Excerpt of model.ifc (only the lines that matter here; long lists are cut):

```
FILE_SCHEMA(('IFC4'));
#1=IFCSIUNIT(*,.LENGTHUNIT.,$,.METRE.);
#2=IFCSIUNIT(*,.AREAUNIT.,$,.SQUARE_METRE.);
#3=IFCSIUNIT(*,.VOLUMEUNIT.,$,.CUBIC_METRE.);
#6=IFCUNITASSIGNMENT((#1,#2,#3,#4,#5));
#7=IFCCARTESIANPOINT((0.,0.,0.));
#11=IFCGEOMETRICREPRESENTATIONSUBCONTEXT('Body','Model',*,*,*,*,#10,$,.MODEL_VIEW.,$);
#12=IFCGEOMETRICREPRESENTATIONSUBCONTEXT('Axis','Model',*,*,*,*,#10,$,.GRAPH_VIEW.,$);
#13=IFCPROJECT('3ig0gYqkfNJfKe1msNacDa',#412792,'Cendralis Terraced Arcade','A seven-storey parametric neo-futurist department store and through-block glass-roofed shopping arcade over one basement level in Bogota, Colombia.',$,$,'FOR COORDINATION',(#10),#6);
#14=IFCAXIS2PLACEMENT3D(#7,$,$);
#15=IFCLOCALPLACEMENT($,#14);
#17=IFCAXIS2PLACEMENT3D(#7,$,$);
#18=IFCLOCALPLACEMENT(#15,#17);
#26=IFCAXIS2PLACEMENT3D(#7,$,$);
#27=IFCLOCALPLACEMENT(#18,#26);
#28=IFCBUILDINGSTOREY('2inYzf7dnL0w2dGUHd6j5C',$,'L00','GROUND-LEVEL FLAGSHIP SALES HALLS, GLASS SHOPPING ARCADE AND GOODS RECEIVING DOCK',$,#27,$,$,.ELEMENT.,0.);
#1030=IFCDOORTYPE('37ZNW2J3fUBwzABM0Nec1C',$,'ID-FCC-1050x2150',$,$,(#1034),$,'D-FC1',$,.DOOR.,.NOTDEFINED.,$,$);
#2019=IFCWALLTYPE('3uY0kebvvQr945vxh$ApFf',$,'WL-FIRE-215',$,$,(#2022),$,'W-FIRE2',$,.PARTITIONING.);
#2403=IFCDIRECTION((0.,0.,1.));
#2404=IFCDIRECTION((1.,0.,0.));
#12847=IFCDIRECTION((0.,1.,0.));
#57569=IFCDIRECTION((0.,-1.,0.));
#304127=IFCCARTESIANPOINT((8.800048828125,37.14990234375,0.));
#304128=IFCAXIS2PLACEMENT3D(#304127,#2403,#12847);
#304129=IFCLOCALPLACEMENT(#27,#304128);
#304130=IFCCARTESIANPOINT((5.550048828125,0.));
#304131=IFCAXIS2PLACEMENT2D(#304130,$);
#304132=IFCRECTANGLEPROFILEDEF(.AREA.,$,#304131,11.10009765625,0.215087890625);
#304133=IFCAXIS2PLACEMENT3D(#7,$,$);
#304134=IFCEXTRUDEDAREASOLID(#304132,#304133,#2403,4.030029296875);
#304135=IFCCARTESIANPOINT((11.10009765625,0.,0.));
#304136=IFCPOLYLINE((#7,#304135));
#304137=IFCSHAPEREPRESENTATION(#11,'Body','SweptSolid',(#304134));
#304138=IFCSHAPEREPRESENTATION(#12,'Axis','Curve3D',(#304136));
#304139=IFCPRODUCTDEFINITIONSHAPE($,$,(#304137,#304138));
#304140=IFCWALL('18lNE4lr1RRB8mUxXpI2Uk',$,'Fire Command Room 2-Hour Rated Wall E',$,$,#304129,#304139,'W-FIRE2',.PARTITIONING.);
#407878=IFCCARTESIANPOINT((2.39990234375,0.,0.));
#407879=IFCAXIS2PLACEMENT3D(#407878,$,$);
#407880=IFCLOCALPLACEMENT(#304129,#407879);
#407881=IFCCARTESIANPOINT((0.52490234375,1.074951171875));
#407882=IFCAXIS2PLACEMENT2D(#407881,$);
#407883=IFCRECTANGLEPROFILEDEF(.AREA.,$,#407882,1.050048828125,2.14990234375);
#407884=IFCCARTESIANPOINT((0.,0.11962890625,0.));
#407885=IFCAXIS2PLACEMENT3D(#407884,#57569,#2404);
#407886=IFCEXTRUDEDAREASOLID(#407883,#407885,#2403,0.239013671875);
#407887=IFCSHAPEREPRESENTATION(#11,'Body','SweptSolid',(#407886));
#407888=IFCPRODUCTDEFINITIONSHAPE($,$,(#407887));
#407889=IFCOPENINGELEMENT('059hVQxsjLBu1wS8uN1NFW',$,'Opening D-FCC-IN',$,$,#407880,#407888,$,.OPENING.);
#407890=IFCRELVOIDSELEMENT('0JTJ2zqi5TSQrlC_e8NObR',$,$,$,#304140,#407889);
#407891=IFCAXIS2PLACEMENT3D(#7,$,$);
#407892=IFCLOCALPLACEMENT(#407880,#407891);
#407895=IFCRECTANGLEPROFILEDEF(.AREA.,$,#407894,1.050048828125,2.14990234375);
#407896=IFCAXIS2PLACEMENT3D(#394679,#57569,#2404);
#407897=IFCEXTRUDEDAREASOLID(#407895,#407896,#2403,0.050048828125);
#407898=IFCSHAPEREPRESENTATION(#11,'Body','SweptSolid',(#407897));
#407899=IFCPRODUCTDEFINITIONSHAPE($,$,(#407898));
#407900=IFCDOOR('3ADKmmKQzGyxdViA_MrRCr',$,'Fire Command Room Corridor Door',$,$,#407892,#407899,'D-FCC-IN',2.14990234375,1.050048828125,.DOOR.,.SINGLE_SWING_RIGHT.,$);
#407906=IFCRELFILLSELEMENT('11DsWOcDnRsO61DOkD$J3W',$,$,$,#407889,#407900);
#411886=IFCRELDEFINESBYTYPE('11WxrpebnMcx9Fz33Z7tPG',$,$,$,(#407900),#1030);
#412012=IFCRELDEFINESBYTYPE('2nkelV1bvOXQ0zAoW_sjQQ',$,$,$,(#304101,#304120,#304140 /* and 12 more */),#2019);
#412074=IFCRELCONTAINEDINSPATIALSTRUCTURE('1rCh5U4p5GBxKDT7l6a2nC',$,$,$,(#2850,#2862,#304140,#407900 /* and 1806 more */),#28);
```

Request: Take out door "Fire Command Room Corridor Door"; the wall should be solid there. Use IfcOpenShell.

```python
import ifcopenshell
import ifcopenshell.api.feature
import ifcopenshell.api.root
import ifcopenshell.geom
import ifcopenshell.util.shape

model = ifcopenshell.open("model.ifc")
settings = ifcopenshell.geom.settings()


def volume(element):
    """Net volume in cubic metres, openings subtracted."""
    shape = ifcopenshell.geom.create_shape(settings, element)
    return ifcopenshell.util.shape.get_volume(shape.geometry)


door = model.by_id(407900)
opening = door.FillsVoids[0].RelatingOpeningElement
wall = opening.VoidsElements[0].RelatingBuildingElement
before = volume(wall)

ifcopenshell.api.root.remove_product(model, product=door)
ifcopenshell.api.feature.remove_feature(model, feature=opening)

after = volume(wall)

print(f"wall volume {before:.3f} -> {after:.3f} m3")

model.write("model-out.ifc")
```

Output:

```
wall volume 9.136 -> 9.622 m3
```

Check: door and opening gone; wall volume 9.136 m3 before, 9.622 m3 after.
